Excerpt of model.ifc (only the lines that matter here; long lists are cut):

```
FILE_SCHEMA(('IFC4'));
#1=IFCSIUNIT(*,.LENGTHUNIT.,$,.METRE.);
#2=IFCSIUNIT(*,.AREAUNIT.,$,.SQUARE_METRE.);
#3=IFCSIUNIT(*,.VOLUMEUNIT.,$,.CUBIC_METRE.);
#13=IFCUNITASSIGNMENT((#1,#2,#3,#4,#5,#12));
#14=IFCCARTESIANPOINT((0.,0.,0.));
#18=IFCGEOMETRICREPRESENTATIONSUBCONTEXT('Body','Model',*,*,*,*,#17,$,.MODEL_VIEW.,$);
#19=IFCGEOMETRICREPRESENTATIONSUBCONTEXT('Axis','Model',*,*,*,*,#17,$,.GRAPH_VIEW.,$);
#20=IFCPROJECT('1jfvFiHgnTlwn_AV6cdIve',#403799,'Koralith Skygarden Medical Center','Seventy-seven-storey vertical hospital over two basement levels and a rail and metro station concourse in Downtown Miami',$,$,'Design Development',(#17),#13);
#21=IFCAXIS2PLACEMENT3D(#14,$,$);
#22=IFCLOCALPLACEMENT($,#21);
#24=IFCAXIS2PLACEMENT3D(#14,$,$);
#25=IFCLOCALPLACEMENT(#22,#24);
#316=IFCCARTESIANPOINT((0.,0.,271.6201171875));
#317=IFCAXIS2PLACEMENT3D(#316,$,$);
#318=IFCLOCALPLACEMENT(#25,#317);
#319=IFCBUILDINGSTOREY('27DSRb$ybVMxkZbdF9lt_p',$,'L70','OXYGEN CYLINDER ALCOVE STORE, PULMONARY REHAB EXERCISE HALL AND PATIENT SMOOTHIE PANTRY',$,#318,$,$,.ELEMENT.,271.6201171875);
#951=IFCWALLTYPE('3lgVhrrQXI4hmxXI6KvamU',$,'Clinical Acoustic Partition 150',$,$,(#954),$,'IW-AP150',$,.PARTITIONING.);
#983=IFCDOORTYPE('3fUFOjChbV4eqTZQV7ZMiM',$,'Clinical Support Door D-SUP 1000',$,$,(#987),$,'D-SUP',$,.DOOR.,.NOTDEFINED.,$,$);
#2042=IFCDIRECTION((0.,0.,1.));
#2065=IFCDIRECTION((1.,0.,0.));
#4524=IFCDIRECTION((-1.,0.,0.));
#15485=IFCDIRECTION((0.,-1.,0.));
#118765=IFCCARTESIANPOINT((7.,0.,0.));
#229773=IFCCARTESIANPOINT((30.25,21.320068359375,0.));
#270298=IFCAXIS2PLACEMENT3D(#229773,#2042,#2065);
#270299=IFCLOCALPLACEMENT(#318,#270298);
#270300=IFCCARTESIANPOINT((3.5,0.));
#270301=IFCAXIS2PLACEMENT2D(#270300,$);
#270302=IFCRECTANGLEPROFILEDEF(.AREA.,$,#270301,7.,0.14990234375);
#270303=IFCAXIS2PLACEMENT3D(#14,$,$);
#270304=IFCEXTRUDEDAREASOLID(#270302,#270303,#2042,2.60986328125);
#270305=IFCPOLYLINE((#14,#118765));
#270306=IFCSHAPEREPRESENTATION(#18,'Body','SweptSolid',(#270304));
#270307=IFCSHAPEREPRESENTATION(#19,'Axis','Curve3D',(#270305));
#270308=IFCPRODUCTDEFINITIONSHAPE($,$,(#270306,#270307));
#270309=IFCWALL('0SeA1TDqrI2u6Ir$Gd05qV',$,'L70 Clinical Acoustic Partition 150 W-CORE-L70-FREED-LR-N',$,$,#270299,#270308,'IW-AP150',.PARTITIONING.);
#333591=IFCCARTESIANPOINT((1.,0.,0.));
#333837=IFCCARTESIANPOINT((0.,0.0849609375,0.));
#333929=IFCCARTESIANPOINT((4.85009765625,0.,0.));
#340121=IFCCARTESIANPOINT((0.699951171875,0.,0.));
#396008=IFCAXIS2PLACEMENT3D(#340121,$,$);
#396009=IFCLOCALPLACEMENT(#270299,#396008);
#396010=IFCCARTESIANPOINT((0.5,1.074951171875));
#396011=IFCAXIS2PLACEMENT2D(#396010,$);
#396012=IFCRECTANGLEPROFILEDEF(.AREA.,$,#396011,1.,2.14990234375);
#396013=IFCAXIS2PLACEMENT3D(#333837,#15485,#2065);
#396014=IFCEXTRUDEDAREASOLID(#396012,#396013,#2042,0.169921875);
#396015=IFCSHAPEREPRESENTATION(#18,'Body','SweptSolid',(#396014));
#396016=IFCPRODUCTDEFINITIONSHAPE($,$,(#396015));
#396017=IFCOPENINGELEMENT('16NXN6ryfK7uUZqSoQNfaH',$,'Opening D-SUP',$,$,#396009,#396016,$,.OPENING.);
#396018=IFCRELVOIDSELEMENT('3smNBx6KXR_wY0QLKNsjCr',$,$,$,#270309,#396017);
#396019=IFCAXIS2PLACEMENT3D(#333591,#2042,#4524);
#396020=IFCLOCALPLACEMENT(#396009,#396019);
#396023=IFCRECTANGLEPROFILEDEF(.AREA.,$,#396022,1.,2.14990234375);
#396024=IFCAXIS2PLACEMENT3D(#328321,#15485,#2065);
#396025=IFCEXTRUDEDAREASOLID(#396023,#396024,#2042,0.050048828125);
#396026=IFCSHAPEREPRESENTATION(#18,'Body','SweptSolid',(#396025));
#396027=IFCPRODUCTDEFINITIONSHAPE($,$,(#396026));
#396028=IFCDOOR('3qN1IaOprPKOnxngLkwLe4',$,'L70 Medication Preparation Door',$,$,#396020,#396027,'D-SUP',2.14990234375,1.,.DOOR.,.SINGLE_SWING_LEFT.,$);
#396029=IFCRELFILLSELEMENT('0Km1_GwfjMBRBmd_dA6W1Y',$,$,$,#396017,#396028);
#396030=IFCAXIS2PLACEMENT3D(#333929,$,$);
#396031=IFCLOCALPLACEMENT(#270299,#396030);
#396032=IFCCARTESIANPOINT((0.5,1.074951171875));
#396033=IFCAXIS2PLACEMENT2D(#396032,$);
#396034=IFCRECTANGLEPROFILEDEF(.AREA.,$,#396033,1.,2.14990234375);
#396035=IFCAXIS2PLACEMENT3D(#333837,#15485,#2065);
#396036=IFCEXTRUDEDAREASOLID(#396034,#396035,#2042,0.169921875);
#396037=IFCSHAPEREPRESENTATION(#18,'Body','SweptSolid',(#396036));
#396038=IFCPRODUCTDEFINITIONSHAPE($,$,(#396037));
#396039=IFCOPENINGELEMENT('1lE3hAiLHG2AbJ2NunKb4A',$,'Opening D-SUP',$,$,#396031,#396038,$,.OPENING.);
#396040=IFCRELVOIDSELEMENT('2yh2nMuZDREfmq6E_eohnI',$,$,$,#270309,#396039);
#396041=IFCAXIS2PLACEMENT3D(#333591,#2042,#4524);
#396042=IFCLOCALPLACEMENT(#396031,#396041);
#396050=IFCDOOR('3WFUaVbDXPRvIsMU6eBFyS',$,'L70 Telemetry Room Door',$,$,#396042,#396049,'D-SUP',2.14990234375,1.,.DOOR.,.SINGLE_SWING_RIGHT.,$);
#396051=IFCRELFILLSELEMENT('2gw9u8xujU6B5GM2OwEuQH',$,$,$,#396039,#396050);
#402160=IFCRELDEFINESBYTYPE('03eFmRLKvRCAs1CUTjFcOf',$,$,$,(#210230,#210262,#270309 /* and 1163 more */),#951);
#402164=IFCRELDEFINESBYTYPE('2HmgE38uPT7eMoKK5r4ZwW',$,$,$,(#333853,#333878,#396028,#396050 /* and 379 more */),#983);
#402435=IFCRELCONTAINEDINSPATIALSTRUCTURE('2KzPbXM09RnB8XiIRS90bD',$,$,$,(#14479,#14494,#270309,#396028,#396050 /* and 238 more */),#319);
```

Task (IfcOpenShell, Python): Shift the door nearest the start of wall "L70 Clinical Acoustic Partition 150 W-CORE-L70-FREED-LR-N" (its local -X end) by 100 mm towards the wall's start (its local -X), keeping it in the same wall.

```python
import ifcopenshell
import ifcopenshell.api.geometry
import ifcopenshell.util.placement
import ifcopenshell.util.unit

model = ifcopenshell.open("model.ifc")
unit_scale = ifcopenshell.util.unit.calculate_unit_scale(model)

door = model.by_guid("3qN1IaOprPKOnxngLkwLe4")
opening = door.FillsVoids[0].RelatingOpeningElement
wall = opening.VoidsElements[0].RelatingBuildingElement

wall_matrix = ifcopenshell.util.placement.get_local_placement(wall.ObjectPlacement)
shift = wall_matrix[:3, 0] * -0.1 / unit_scale
before = ifcopenshell.util.placement.get_local_placement(door.ObjectPlacement)[:3, 3].copy()

# The door is placed relative to its opening, so it follows when the opening moves.
matrix = ifcopenshell.util.placement.get_local_placement(opening.ObjectPlacement)
matrix[:3, 3] += shift
ifcopenshell.api.geometry.edit_object_placement(
    model, product=opening, matrix=matrix, is_si=False, should_transform_children=True
)

after = ifcopenshell.util.placement.get_local_placement(door.ObjectPlacement)[:3, 3]
print("door moved by", (after - before).round(3) + 0.0)

model.write("model_v2.ifc")
```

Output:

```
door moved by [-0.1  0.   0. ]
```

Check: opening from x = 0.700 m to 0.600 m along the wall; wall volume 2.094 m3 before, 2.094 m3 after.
